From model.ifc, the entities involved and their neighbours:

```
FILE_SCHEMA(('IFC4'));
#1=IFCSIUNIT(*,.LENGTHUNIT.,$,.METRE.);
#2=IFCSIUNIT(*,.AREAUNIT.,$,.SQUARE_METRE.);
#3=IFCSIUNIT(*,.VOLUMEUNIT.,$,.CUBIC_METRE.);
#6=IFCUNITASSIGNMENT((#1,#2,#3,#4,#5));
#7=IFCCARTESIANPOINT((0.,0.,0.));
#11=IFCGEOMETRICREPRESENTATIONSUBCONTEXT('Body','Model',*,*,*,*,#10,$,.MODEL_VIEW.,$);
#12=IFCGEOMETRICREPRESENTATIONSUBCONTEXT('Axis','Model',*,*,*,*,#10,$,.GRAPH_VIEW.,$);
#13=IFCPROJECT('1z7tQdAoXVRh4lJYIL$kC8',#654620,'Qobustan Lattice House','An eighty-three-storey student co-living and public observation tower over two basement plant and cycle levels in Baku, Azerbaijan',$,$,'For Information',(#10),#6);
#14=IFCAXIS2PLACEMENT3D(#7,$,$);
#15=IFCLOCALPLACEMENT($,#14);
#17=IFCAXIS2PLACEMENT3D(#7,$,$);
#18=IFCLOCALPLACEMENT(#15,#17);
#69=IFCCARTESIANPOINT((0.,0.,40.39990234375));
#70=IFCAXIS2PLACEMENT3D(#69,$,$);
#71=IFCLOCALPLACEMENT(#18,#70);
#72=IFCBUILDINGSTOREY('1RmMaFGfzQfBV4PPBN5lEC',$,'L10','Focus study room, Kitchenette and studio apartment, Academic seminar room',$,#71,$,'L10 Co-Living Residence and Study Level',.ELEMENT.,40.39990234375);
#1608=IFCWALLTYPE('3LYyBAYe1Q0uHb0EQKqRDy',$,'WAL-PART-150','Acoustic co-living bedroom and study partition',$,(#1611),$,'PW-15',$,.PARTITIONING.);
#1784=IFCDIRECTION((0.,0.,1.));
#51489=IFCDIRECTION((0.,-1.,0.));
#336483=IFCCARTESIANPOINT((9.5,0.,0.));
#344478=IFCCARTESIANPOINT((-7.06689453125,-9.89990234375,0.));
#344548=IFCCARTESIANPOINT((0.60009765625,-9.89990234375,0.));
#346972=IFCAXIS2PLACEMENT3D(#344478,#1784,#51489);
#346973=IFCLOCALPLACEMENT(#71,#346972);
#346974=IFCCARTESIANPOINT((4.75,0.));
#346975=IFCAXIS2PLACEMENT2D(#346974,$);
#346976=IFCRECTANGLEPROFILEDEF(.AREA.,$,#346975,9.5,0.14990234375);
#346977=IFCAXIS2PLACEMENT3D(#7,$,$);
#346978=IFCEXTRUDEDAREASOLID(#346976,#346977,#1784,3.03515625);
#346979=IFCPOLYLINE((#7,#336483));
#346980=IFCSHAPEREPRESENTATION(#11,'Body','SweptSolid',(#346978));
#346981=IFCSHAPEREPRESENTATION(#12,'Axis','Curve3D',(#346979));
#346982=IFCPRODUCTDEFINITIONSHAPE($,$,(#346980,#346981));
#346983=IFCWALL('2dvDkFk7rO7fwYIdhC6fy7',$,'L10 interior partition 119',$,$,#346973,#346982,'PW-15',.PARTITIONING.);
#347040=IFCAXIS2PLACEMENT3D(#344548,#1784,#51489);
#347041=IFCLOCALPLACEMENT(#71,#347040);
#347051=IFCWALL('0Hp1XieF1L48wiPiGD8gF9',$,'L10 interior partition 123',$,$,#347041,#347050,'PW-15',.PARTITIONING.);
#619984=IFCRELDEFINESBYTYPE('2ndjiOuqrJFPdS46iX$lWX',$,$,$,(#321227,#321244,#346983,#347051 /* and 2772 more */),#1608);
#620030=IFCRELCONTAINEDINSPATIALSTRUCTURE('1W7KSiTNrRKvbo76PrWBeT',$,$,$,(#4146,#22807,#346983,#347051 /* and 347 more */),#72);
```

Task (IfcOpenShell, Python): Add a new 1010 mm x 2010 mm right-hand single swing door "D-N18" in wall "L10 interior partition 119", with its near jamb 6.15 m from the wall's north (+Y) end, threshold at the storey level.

```python
import numpy as np
import ifcopenshell
import ifcopenshell.api.feature
import ifcopenshell.api.geometry
import ifcopenshell.api.root
import ifcopenshell.api.spatial
import ifcopenshell.geom
import ifcopenshell.util.element
import ifcopenshell.util.placement
import ifcopenshell.util.representation
import ifcopenshell.util.shape
import ifcopenshell.util.unit

model = ifcopenshell.open("model.ifc")
unit_scale = ifcopenshell.util.unit.calculate_unit_scale(model)
settings = ifcopenshell.geom.settings()


def volume(element):
    """Net volume in cubic metres, openings subtracted."""
    shape = ifcopenshell.geom.create_shape(settings, element)
    return ifcopenshell.util.shape.get_volume(shape.geometry)


wall = model.by_guid("2dvDkFk7rO7fwYIdhC6fy7")
storey = ifcopenshell.util.element.get_container(wall, ifc_class="IfcBuildingStorey")
context = ifcopenshell.util.representation.get_context(model, "Model", "Body", "MODEL_VIEW")
before = volume(wall)

width, height, from_end, sill = 1.01, 2.01, 6.15, 0.0  # metres

# The wall runs along its own X axis, and the end named is its -X end.
wall_shape = ifcopenshell.geom.create_shape(settings, wall)
x, y, z = ifcopenshell.util.shape.get_vertices(wall_shape.geometry).T
start = x.min() + from_end
face, thickness = float(y.min()), float(y.max() - y.min())
wall_matrix = ifcopenshell.util.placement.get_local_placement(wall.ObjectPlacement)
level = ifcopenshell.util.placement.get_local_placement(storey.ObjectPlacement)[2, 3]


def in_wall(x, y):
    """Placement at x, y metres in the wall's axes, at sill height."""
    matrix = wall_matrix.copy()
    matrix[:, 3] = wall_matrix @ np.array([x / unit_scale, y / unit_scale, 0.0, 1.0])
    matrix[2, 3] = level + sill / unit_scale
    return matrix


# Opening: a box that overshoots both wall faces by 50 mm.
opening = ifcopenshell.api.root.create_entity(model, ifc_class="IfcOpeningElement", predefined_type="OPENING")
box = ifcopenshell.api.geometry.add_wall_representation(
    model, context=context, length=width, height=height, thickness=thickness + 0.1
)
ifcopenshell.api.geometry.assign_representation(model, product=opening, representation=box)
ifcopenshell.api.geometry.edit_object_placement(model, product=opening, matrix=in_wall(start, face - 0.05), is_si=False)
ifcopenshell.api.feature.add_feature(model, feature=opening, element=wall)

door = ifcopenshell.api.root.create_entity(model, ifc_class="IfcDoor", name="D-N18", predefined_type="DOOR")
door.OverallWidth, door.OverallHeight = width / unit_scale, height / unit_scale
door.OperationType = "SINGLE_SWING_RIGHT"
body = ifcopenshell.api.geometry.add_door_representation(
    model,
    context=context,
    overall_width=door.OverallWidth,
    overall_height=door.OverallHeight,
    operation_type="SINGLE_SWING_RIGHT",
    lining_properties={"LiningDepth": thickness / unit_scale, "ThresholdDepth": thickness / unit_scale},
)
ifcopenshell.api.geometry.assign_representation(model, product=door, representation=body)
ifcopenshell.api.spatial.assign_container(model, products=[door], relating_structure=storey)
ifcopenshell.api.feature.add_filling(model, opening=opening, element=door)

# The lining spans the wall, so the door starts at the wall face.
ifcopenshell.api.geometry.edit_object_placement(model, product=door, matrix=in_wall(start, face), is_si=False)

after = volume(wall)

print(f"wall volume {before:.3f} -> {after:.3f} m3")

model.write("model_updated.ifc")
```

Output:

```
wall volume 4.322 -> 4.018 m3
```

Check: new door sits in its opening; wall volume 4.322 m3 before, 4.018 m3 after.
